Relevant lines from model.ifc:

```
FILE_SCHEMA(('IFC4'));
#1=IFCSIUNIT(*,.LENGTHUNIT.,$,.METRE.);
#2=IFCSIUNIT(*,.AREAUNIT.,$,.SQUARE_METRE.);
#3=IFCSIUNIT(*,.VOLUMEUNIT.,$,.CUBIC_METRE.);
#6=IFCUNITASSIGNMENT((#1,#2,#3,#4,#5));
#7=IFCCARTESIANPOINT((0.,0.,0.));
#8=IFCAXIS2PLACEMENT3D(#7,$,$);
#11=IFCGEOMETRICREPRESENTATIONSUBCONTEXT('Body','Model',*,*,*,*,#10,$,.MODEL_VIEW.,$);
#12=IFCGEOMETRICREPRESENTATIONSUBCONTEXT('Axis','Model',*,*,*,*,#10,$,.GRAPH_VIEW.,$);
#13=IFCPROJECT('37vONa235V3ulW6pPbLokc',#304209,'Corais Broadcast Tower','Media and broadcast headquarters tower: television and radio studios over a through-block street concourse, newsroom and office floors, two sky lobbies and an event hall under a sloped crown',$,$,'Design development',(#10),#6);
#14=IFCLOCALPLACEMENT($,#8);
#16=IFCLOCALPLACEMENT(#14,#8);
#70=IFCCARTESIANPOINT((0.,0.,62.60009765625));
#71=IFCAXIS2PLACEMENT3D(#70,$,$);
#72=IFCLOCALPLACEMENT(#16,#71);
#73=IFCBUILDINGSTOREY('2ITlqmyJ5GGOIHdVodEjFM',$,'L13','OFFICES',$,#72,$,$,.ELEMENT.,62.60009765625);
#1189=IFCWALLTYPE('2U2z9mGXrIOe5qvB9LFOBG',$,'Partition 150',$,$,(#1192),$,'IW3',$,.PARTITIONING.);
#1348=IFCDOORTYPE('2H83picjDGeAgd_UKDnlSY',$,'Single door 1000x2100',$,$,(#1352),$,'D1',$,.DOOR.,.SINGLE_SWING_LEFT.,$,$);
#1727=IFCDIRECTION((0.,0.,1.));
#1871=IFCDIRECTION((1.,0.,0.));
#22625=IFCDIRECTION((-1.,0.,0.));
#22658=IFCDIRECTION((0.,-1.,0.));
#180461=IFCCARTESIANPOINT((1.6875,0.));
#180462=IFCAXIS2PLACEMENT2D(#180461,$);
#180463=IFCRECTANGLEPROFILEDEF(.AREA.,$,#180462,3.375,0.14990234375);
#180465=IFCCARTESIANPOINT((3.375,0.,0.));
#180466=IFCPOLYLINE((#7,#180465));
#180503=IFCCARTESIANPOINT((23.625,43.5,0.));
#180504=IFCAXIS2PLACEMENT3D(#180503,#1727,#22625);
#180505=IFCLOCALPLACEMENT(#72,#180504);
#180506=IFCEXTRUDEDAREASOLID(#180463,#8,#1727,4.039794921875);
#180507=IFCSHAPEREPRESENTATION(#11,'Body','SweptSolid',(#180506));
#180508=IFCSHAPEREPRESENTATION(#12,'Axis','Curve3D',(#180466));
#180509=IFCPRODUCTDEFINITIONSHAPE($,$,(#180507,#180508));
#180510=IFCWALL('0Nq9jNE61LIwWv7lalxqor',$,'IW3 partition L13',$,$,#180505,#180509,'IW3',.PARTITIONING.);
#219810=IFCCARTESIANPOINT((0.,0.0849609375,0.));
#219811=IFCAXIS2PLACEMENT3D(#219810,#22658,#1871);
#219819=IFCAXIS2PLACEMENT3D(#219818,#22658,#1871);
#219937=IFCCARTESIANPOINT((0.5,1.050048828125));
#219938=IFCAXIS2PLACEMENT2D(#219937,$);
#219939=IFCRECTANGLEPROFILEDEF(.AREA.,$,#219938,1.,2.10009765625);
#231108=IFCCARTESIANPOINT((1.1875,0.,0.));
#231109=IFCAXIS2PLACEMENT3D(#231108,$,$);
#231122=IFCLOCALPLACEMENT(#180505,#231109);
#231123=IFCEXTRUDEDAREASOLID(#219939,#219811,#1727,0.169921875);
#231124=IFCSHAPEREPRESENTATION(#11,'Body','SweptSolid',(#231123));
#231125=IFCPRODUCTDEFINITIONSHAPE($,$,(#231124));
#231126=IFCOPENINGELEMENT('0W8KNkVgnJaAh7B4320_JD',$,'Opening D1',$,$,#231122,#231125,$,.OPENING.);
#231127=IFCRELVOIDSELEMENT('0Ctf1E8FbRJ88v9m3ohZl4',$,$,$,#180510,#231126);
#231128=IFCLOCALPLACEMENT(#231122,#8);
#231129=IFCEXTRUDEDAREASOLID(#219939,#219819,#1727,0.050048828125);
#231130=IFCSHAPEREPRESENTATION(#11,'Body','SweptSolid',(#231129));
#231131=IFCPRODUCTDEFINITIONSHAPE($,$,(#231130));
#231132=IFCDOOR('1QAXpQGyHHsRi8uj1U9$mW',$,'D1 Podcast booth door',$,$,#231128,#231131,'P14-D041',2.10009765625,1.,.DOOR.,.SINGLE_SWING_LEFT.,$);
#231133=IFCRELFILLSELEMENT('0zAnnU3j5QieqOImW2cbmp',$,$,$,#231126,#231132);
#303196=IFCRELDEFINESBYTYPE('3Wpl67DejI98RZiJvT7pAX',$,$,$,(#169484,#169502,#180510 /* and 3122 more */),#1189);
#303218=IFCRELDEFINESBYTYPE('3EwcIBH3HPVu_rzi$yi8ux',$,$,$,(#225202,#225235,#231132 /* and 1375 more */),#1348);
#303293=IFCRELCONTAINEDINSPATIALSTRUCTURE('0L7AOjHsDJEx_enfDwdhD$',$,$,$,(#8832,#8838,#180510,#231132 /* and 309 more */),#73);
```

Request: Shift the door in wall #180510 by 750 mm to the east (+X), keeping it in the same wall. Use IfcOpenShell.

```python
import ifcopenshell
import ifcopenshell.api.geometry
import ifcopenshell.util.placement
import ifcopenshell.util.unit

model = ifcopenshell.open("model.ifc")
unit_scale = ifcopenshell.util.unit.calculate_unit_scale(model)

door = model.by_guid("1QAXpQGyHHsRi8uj1U9$mW")
opening = door.FillsVoids[0].RelatingOpeningElement
wall = opening.VoidsElements[0].RelatingBuildingElement

wall_matrix = ifcopenshell.util.placement.get_local_placement(wall.ObjectPlacement)
shift = wall_matrix[:3, 0] * -0.75 / unit_scale
before = ifcopenshell.util.placement.get_local_placement(door.ObjectPlacement)[:3, 3].copy()

# The door is placed relative to its opening, so it follows when the opening moves.
matrix = ifcopenshell.util.placement.get_local_placement(opening.ObjectPlacement)
matrix[:3, 3] += shift
ifcopenshell.api.geometry.edit_object_placement(
    model, product=opening, matrix=matrix, is_si=False, should_transform_children=True
)

after = ifcopenshell.util.placement.get_local_placement(door.ObjectPlacement)[:3, 3]
print("door moved by", (after - before).round(3) + 0.0)

model.write("model-out.ifc")
```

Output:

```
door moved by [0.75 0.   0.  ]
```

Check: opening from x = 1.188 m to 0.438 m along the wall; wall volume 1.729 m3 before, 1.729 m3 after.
